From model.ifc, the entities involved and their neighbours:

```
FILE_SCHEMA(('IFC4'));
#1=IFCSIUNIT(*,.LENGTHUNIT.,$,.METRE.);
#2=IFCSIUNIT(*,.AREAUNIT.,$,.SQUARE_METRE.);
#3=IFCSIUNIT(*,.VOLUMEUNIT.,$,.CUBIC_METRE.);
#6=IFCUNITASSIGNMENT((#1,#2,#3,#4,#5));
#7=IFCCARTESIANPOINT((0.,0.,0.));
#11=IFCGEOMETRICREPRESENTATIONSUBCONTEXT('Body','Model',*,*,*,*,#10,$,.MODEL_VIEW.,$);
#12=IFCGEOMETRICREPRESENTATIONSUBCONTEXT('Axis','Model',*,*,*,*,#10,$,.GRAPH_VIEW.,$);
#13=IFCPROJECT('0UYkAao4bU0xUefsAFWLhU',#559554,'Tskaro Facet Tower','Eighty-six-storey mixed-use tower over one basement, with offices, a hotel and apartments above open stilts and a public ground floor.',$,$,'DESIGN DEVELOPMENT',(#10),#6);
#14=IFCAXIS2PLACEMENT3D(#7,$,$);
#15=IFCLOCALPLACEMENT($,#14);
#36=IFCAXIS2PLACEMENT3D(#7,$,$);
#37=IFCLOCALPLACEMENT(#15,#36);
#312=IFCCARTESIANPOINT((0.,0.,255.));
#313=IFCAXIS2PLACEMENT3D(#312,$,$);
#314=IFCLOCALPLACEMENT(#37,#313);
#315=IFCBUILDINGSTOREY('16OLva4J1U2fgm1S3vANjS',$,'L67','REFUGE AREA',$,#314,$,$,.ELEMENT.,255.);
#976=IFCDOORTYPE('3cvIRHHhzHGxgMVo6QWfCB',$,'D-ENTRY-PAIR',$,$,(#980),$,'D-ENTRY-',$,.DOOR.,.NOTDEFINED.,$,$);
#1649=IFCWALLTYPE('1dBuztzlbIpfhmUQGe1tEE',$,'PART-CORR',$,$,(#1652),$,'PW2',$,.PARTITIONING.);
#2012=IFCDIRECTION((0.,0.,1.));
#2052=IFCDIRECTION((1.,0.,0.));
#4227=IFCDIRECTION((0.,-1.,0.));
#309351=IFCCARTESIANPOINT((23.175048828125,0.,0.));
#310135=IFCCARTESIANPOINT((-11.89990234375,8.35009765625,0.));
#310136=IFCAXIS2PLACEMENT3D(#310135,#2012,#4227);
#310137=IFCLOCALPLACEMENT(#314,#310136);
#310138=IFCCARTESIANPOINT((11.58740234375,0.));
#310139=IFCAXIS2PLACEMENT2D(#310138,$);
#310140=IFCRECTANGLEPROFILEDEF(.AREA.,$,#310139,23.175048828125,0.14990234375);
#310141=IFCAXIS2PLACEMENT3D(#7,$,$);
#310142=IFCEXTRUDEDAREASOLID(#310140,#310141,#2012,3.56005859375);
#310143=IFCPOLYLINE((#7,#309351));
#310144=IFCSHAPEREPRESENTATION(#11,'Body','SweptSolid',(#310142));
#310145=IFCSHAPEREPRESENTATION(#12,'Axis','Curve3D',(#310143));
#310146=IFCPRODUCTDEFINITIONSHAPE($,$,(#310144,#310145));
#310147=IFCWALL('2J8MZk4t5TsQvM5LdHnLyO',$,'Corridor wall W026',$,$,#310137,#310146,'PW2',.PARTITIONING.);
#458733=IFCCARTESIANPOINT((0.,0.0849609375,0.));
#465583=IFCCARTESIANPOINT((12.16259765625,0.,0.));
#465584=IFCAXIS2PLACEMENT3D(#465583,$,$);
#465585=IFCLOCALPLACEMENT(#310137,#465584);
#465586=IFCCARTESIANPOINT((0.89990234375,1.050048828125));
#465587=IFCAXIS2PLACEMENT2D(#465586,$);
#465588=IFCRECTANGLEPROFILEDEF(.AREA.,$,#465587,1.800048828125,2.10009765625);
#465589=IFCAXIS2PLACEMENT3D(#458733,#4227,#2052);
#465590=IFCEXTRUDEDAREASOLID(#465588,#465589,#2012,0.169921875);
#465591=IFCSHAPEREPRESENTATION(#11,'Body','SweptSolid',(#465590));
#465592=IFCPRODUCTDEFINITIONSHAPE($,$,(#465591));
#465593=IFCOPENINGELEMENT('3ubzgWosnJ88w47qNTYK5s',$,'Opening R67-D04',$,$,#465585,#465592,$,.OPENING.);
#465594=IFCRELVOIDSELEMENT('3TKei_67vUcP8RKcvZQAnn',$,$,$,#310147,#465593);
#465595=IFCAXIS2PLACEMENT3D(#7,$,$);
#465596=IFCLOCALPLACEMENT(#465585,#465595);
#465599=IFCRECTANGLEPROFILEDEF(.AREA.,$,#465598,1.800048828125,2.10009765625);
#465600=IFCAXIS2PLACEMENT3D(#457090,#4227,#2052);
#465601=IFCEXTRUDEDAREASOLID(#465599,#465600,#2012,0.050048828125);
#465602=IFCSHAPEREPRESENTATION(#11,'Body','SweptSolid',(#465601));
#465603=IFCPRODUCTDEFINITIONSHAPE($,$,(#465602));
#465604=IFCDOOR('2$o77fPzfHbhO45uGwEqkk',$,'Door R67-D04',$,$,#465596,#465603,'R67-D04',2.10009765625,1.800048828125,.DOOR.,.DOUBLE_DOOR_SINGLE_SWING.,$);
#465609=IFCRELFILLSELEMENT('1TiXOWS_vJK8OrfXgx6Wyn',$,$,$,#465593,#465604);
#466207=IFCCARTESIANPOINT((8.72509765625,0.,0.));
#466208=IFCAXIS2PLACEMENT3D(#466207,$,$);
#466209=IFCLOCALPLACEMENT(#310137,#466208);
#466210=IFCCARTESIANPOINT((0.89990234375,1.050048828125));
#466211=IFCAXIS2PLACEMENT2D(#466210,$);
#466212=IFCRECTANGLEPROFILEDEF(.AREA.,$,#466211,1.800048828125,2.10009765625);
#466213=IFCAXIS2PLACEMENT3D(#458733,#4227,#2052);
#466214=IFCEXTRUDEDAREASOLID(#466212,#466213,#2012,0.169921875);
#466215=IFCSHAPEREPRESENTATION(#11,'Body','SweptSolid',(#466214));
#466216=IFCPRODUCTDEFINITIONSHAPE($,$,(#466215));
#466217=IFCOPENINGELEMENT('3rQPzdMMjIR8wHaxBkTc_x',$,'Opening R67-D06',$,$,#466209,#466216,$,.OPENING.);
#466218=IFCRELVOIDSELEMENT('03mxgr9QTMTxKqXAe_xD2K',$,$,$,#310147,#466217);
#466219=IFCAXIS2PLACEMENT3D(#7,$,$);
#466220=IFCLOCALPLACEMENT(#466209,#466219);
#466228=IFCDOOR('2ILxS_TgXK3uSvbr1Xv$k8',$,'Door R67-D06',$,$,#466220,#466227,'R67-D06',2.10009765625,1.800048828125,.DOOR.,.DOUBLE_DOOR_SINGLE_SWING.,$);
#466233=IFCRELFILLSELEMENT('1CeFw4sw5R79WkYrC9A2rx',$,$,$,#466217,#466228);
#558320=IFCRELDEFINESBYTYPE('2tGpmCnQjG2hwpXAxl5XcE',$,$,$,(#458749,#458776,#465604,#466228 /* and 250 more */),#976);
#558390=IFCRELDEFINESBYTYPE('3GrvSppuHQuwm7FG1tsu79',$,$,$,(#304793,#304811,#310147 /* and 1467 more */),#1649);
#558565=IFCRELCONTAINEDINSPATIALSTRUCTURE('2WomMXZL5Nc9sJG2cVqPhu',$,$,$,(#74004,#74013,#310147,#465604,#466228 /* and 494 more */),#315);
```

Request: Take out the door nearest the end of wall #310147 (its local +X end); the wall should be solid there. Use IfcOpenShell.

```python
import ifcopenshell
import ifcopenshell.api.feature
import ifcopenshell.api.root
import ifcopenshell.geom
import ifcopenshell.util.shape

model = ifcopenshell.open("model.ifc")
settings = ifcopenshell.geom.settings()


def volume(element):
    """Net volume in cubic metres, openings subtracted."""
    shape = ifcopenshell.geom.create_shape(settings, element)
    return ifcopenshell.util.shape.get_volume(shape.geometry)


door = model.by_guid("2$o77fPzfHbhO45uGwEqkk")
opening = door.FillsVoids[0].RelatingOpeningElement
wall = opening.VoidsElements[0].RelatingBuildingElement
before = volume(wall)

ifcopenshell.api.root.remove_product(model, product=door)
ifcopenshell.api.feature.remove_feature(model, feature=opening)

after = volume(wall)

print(f"wall volume {before:.3f} -> {after:.3f} m3")

model.write("model-out.ifc")
```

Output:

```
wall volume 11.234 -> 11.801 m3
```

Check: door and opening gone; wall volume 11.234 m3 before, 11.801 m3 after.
